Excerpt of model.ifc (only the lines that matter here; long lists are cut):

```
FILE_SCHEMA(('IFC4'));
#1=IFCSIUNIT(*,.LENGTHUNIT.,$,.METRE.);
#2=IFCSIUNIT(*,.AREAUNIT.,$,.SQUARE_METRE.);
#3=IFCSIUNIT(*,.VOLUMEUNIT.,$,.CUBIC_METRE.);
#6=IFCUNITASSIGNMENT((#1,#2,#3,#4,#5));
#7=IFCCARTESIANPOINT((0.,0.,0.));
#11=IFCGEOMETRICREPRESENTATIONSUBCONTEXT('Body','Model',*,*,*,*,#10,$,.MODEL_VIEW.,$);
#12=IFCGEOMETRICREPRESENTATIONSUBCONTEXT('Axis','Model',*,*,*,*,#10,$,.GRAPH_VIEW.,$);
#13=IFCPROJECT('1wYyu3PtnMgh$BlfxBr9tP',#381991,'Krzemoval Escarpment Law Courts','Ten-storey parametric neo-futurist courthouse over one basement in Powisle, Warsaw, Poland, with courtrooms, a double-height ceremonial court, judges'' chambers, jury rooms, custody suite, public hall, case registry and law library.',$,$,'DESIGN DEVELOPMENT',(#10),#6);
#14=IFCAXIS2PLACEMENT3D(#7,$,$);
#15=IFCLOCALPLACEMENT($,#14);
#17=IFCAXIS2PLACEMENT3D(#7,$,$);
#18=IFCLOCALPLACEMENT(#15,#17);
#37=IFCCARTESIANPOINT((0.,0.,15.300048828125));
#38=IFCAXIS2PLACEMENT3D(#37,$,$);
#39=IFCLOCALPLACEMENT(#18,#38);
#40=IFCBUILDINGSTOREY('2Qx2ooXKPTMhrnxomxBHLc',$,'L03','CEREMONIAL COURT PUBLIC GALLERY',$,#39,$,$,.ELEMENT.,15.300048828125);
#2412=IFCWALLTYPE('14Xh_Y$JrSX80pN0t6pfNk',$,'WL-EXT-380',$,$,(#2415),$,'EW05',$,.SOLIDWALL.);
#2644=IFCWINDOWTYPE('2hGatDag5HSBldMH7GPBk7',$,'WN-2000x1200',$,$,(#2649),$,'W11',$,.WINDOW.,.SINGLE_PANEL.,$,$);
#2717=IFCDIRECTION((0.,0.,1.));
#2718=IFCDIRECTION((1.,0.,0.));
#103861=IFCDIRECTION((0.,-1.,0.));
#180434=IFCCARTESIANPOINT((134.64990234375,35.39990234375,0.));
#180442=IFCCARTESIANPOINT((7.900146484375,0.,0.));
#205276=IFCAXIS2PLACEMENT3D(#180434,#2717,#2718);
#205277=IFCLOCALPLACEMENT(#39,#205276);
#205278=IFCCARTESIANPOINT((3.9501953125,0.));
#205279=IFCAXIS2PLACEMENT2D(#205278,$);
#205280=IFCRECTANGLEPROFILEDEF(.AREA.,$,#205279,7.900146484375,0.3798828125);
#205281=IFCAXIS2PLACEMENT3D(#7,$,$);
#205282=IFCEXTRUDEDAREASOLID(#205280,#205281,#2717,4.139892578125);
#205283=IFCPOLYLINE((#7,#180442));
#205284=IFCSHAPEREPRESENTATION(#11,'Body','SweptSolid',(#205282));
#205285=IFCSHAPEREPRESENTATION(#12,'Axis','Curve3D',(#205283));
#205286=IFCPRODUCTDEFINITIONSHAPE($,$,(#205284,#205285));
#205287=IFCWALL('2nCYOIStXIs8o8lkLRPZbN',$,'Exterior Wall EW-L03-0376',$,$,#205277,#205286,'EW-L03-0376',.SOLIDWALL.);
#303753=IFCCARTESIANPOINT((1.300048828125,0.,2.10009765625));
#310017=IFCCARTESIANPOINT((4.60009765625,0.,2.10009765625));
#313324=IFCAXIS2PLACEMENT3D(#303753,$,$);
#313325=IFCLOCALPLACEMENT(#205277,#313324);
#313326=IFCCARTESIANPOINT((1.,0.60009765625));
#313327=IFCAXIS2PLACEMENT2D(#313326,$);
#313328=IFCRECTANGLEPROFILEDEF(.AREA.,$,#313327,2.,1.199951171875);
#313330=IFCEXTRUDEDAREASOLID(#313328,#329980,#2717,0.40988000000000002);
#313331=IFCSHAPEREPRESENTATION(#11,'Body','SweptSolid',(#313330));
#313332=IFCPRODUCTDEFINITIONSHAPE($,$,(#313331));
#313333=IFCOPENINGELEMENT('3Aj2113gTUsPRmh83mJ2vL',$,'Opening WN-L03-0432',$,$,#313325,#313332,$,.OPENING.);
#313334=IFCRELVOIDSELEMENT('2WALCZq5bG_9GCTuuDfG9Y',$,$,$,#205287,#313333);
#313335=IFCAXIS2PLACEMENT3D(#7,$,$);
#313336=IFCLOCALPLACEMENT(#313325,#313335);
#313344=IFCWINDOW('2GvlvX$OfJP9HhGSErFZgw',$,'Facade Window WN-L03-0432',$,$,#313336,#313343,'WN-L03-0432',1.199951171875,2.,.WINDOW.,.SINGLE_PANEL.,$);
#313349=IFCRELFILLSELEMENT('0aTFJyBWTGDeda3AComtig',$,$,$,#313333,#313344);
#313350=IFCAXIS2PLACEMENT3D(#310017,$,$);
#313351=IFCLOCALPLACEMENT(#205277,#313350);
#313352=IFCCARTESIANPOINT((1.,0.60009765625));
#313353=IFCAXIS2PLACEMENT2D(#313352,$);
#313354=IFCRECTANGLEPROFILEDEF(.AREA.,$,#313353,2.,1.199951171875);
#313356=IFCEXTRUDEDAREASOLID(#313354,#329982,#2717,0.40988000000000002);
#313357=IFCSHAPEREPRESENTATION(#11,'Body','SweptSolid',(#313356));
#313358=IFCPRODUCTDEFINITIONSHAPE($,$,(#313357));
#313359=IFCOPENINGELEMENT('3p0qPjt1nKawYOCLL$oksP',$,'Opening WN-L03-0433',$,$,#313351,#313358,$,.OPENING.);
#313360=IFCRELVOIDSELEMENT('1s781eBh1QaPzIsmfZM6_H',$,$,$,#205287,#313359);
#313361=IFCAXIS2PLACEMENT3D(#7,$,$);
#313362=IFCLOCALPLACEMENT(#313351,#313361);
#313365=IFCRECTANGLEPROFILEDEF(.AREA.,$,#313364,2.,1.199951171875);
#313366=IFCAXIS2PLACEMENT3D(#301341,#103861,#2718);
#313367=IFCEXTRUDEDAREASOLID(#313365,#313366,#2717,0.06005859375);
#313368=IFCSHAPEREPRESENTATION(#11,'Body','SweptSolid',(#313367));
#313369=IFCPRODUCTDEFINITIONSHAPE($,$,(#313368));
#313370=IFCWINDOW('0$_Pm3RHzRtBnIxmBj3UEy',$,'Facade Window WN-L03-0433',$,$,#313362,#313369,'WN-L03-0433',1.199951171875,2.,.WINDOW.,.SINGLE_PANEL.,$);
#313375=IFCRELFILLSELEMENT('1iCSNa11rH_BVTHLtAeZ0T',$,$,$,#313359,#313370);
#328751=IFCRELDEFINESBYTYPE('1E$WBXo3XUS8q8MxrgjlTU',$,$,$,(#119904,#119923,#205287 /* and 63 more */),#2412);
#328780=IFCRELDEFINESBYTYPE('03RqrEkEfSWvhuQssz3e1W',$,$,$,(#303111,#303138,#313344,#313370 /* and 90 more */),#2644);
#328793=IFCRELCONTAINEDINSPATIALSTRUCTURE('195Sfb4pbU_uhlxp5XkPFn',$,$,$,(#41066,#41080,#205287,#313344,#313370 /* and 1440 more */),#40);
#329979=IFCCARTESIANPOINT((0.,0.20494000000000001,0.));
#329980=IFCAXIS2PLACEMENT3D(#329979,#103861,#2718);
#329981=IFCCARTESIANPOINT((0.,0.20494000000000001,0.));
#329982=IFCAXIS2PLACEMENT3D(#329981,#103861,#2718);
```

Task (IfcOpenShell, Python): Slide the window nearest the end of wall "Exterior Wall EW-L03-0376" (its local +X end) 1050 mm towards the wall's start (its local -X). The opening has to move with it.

```python
import ifcopenshell
import ifcopenshell.api.geometry
import ifcopenshell.util.placement
import ifcopenshell.util.unit

model = ifcopenshell.open("model.ifc")
unit_scale = ifcopenshell.util.unit.calculate_unit_scale(model)

window = model.by_guid("0$_Pm3RHzRtBnIxmBj3UEy")
opening = window.FillsVoids[0].RelatingOpeningElement
wall = opening.VoidsElements[0].RelatingBuildingElement

wall_matrix = ifcopenshell.util.placement.get_local_placement(wall.ObjectPlacement)
shift = wall_matrix[:3, 0] * -1.05 / unit_scale
before = ifcopenshell.util.placement.get_local_placement(window.ObjectPlacement)[:3, 3].copy()

# The window is placed relative to its opening, so it follows when the opening moves.
matrix = ifcopenshell.util.placement.get_local_placement(opening.ObjectPlacement)
matrix[:3, 3] += shift
ifcopenshell.api.geometry.edit_object_placement(
    model, product=opening, matrix=matrix, is_si=False, should_transform_children=True
)

after = ifcopenshell.util.placement.get_local_placement(window.ObjectPlacement)[:3, 3]
print("window moved by", (after - before).round(3) + 0.0)

model.write("model_updated.ifc")
```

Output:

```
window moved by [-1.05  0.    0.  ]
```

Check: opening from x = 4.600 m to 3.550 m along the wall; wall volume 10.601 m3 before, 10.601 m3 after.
